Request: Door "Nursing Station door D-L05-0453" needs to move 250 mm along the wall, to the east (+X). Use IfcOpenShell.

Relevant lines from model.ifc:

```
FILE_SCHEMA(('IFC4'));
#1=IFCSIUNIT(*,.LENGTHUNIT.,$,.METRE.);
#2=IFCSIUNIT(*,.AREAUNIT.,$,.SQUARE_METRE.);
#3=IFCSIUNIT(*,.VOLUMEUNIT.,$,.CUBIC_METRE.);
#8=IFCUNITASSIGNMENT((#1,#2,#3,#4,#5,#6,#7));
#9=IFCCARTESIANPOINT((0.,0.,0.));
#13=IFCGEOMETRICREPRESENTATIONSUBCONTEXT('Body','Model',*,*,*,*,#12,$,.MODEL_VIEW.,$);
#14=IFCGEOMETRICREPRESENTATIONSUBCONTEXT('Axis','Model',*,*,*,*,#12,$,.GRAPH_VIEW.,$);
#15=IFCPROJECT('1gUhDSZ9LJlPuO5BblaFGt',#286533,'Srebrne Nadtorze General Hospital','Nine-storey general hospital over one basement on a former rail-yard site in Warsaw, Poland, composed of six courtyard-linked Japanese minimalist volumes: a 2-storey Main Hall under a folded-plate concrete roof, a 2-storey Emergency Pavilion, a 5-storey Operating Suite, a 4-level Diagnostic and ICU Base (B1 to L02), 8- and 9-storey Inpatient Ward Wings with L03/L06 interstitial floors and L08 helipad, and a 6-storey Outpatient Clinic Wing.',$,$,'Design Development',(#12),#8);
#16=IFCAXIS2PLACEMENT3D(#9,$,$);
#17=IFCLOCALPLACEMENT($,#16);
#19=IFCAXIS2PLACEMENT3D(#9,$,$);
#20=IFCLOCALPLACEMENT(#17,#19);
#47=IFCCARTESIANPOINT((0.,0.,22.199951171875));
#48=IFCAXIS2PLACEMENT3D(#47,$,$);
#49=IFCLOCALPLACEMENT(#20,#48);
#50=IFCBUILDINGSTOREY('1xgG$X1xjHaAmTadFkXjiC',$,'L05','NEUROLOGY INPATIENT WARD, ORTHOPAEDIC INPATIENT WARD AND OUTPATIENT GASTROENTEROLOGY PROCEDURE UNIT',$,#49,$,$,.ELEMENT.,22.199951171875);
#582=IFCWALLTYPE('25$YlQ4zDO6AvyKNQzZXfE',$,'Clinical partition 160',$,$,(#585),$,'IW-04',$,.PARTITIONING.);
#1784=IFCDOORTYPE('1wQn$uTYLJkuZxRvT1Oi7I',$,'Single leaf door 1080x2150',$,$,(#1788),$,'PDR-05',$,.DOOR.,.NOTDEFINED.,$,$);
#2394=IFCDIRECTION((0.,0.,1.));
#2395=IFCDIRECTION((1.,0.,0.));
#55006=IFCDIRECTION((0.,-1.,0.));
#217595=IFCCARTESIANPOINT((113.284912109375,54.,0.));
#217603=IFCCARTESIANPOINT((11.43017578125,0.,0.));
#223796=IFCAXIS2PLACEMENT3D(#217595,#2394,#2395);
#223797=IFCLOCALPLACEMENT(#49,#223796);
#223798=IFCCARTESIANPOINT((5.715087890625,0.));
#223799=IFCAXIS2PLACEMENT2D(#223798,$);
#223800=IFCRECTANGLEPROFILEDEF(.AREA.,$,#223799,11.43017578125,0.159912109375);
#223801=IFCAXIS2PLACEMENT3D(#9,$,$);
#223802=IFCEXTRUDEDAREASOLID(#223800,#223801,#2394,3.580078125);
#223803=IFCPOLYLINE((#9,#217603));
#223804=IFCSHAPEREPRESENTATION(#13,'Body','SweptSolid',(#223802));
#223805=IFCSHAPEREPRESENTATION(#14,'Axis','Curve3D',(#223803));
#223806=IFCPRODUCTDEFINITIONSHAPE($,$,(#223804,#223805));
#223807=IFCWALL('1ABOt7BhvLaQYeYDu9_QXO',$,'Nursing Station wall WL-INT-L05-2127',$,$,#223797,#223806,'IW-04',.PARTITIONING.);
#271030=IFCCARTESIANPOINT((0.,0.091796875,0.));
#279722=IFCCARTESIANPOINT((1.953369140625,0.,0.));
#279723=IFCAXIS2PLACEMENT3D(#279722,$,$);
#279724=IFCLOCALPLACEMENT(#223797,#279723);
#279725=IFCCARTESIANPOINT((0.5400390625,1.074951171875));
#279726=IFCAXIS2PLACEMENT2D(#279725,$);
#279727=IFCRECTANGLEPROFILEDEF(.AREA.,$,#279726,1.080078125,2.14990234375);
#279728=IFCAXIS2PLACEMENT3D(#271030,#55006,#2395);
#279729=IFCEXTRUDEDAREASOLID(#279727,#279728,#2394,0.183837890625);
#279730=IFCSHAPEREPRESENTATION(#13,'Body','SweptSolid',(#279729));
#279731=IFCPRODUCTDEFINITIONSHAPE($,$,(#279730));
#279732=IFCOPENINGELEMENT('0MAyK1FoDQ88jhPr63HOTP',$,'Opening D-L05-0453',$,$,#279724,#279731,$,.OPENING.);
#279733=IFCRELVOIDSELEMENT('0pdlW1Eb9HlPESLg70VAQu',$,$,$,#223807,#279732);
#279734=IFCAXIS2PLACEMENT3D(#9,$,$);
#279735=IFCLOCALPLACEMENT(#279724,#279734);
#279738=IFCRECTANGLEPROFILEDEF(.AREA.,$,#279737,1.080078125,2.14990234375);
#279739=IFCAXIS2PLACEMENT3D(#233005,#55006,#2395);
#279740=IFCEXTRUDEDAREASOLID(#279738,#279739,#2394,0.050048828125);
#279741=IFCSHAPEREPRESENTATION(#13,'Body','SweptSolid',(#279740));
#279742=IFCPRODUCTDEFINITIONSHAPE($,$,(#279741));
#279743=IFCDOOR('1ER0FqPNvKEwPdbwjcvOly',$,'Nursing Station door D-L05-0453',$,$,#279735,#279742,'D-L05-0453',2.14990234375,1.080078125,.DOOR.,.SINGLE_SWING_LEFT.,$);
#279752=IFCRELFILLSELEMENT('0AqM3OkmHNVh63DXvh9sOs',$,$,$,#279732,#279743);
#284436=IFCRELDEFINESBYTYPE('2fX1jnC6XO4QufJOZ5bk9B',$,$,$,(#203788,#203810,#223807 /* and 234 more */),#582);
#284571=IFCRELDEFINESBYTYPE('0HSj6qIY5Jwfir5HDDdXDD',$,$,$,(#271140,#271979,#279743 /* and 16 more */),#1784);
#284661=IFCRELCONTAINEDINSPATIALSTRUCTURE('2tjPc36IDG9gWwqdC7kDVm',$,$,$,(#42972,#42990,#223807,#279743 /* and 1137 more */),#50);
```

```python
import ifcopenshell
import ifcopenshell.api.geometry
import ifcopenshell.util.placement

model = ifcopenshell.open("model.ifc")

door = model.by_guid("1ER0FqPNvKEwPdbwjcvOly")
opening = door.FillsVoids[0].RelatingOpeningElement
wall = opening.VoidsElements[0].RelatingBuildingElement

wall_matrix = ifcopenshell.util.placement.get_local_placement(wall.ObjectPlacement)
shift = wall_matrix[:3, 0] * 0.25
before = ifcopenshell.util.placement.get_local_placement(door.ObjectPlacement)[:3, 3].copy()

# The door is placed relative to its opening, so it follows when the opening moves.
matrix = ifcopenshell.util.placement.get_local_placement(opening.ObjectPlacement)
matrix[:3, 3] += shift
ifcopenshell.api.geometry.edit_object_placement(
    model, product=opening, matrix=matrix, is_si=False, should_transform_children=True
)

after = ifcopenshell.util.placement.get_local_placement(door.ObjectPlacement)[:3, 3]
print("door moved by", (after - before).round(3) + 0.0)

model.write("model_edited.ifc")
```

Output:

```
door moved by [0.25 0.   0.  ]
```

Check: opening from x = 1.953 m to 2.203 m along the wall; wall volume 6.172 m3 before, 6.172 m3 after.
